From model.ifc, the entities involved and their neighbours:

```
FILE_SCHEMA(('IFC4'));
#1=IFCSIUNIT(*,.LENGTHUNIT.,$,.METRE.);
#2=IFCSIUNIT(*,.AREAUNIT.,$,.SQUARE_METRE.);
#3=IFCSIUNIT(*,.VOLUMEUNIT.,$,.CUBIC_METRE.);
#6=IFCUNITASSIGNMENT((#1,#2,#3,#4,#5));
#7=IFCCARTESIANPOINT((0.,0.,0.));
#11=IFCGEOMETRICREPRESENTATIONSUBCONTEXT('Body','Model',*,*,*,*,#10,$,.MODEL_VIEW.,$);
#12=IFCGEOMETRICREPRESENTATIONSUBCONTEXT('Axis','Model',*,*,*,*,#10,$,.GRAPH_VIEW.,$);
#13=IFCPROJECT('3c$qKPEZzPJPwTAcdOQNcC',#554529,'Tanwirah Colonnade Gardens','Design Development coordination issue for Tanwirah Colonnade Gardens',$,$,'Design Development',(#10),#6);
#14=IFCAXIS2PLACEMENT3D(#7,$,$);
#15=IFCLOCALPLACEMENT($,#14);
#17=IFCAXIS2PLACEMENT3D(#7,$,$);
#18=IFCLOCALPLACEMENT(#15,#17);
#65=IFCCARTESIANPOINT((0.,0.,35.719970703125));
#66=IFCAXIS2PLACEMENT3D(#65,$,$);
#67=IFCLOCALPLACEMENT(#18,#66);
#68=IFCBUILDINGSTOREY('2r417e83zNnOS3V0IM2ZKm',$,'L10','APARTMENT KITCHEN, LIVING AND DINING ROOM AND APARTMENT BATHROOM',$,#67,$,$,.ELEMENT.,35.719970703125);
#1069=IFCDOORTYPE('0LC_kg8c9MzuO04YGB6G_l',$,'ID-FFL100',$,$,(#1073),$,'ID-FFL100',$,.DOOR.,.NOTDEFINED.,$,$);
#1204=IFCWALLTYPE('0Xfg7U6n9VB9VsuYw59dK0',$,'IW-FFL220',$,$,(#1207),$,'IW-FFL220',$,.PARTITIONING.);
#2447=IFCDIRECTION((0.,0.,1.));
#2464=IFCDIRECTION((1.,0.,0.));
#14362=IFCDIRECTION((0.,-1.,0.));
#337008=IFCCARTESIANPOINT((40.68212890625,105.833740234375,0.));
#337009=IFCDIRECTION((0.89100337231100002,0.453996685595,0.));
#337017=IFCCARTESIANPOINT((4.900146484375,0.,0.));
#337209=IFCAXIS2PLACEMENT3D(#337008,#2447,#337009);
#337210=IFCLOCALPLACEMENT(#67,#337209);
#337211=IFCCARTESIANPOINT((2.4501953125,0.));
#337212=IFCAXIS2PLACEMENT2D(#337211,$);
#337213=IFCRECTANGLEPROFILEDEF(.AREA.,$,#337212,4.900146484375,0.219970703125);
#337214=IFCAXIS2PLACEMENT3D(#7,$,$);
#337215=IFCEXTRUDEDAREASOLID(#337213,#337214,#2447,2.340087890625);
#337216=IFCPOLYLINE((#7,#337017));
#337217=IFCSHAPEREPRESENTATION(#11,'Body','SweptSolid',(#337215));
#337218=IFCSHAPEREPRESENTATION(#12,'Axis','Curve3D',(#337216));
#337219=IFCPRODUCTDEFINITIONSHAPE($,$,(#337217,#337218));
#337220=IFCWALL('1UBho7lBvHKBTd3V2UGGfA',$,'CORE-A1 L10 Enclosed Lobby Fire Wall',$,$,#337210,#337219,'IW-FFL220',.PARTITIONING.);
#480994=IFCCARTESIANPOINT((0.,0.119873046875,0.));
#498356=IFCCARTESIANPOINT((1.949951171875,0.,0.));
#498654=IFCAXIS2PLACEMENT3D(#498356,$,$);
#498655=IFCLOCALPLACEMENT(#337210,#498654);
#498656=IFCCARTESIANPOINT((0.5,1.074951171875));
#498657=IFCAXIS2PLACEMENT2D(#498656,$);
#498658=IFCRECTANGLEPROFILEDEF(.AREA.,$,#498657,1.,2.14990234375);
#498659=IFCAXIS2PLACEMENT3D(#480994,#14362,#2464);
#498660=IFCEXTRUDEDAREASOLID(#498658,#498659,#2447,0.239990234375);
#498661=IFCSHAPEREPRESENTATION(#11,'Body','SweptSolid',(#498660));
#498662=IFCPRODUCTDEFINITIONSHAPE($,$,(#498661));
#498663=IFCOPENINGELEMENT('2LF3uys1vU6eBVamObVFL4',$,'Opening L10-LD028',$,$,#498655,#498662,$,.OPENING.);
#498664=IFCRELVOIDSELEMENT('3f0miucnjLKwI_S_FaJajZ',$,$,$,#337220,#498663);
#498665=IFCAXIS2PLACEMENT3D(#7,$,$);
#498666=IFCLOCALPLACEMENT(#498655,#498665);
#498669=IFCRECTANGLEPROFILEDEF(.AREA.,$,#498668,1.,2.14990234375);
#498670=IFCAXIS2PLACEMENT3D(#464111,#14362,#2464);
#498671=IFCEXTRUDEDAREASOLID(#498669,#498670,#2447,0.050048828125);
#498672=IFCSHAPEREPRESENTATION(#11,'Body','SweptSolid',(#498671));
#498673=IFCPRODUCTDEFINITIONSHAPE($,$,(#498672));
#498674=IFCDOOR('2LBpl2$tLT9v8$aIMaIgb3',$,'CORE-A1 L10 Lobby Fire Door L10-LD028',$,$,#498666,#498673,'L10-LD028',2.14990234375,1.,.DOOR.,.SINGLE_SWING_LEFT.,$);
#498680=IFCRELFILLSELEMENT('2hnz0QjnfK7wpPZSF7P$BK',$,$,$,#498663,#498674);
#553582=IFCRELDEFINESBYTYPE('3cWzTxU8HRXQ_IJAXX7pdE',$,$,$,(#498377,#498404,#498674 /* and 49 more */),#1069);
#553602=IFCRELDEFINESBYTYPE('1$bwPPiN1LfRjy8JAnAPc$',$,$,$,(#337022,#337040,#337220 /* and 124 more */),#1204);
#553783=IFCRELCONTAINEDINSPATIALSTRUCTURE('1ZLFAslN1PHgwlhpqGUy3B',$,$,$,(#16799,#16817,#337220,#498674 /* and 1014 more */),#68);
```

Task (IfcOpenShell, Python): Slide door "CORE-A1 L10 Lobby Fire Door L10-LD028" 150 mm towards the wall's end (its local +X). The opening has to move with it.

```python
import ifcopenshell
import ifcopenshell.api.geometry
import ifcopenshell.util.placement

model = ifcopenshell.open("model.ifc")

door = model.by_guid("2LBpl2$tLT9v8$aIMaIgb3")
opening = door.FillsVoids[0].RelatingOpeningElement
wall = opening.VoidsElements[0].RelatingBuildingElement

wall_matrix = ifcopenshell.util.placement.get_local_placement(wall.ObjectPlacement)
shift = wall_matrix[:3, 0] * 0.15
before = ifcopenshell.util.placement.get_local_placement(door.ObjectPlacement)[:3, 3].copy()

# The door is placed relative to its opening, so it follows when the opening moves.
matrix = ifcopenshell.util.placement.get_local_placement(opening.ObjectPlacement)
matrix[:3, 3] += shift
ifcopenshell.api.geometry.edit_object_placement(
    model, product=opening, matrix=matrix, is_si=False, should_transform_children=True
)

after = ifcopenshell.util.placement.get_local_placement(door.ObjectPlacement)[:3, 3]
print("door moved by", (after - before).round(3) + 0.0)

model.write("model-out.ifc")
```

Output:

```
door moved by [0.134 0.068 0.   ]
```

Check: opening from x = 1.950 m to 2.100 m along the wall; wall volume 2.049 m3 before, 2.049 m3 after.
